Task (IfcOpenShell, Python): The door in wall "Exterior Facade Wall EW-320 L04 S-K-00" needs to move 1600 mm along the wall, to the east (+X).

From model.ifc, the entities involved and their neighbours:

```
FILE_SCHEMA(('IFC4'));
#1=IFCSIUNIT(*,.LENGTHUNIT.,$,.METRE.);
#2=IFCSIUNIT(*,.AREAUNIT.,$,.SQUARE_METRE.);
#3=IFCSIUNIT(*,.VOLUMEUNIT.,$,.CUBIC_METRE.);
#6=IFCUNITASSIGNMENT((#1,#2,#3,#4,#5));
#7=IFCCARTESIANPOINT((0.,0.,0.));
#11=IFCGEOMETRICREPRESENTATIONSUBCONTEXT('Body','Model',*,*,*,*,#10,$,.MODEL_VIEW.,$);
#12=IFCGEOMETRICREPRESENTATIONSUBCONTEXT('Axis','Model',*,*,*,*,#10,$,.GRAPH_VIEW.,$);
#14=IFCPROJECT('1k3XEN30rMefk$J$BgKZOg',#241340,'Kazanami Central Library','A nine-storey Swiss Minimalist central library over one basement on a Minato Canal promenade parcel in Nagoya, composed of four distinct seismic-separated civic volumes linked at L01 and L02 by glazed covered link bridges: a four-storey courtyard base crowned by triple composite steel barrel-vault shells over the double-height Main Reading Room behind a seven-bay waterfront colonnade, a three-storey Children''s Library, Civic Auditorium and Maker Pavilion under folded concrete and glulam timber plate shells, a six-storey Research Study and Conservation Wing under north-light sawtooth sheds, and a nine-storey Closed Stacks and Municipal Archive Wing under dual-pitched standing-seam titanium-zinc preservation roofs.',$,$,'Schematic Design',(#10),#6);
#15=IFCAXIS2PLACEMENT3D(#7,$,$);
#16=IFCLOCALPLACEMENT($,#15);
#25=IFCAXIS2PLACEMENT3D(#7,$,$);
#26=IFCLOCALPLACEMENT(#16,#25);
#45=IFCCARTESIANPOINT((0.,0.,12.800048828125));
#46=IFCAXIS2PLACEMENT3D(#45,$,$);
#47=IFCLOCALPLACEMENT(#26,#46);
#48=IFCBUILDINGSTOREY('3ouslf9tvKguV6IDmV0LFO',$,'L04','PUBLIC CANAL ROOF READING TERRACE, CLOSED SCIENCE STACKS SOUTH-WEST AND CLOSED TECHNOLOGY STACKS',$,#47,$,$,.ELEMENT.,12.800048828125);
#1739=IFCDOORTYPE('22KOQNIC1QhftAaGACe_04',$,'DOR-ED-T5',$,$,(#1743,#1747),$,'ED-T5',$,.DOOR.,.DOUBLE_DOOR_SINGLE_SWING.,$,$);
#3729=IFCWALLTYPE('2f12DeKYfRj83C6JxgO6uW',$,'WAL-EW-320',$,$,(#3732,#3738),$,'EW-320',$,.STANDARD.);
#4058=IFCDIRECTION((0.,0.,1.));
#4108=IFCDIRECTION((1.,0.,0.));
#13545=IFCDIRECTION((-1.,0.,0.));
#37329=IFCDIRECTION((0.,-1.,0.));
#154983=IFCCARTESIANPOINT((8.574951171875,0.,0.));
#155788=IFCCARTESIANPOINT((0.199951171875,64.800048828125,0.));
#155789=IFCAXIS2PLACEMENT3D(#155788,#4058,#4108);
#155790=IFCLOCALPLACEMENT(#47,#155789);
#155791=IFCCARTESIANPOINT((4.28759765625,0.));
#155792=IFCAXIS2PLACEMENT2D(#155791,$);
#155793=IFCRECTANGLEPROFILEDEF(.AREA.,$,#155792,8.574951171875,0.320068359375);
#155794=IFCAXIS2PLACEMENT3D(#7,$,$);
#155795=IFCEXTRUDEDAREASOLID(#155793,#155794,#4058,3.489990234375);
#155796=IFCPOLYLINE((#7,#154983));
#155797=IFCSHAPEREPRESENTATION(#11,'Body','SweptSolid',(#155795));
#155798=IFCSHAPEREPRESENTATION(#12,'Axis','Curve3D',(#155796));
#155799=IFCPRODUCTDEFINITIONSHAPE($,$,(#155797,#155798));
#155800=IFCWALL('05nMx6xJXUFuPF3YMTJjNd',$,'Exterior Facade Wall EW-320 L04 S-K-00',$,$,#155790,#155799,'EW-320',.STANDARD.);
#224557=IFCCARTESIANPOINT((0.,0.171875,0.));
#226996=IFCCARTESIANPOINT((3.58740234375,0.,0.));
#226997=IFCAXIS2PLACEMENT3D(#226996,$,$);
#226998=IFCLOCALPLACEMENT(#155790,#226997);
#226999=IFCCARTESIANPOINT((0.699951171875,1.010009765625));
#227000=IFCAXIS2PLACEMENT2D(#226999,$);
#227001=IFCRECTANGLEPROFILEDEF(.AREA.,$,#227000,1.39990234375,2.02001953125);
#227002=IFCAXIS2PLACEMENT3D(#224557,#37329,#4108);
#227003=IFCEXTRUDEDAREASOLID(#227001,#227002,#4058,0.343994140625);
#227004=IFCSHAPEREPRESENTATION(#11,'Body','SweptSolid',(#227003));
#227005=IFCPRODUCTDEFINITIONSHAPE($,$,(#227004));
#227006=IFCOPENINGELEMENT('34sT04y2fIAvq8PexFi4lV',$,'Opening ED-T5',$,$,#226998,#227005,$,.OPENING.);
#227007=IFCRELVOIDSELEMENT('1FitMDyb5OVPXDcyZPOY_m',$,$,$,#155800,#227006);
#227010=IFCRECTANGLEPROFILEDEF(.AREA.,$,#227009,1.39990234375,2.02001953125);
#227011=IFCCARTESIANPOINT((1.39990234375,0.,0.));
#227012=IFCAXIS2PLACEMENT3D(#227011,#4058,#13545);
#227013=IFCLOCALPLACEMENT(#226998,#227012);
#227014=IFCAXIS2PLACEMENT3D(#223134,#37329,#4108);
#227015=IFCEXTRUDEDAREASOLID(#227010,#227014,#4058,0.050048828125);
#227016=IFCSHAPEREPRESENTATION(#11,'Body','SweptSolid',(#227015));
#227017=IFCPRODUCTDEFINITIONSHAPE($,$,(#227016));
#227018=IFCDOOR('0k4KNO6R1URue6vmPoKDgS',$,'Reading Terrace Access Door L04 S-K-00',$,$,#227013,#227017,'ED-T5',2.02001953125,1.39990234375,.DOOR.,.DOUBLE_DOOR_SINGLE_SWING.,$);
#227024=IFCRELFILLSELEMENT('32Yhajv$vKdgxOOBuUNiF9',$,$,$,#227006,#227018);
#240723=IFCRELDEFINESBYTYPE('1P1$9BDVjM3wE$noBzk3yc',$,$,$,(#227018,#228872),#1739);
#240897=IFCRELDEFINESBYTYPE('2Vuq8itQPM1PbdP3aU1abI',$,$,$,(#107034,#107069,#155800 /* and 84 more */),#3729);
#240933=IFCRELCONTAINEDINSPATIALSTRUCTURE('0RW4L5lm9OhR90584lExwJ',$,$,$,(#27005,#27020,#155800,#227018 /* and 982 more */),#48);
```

```python
import ifcopenshell
import ifcopenshell.api.geometry
import ifcopenshell.util.placement
import ifcopenshell.util.unit

model = ifcopenshell.open("model.ifc")
unit_scale = ifcopenshell.util.unit.calculate_unit_scale(model)

door = model.by_id(227018)
opening = door.FillsVoids[0].RelatingOpeningElement
wall = opening.VoidsElements[0].RelatingBuildingElement

wall_matrix = ifcopenshell.util.placement.get_local_placement(wall.ObjectPlacement)
shift = wall_matrix[:3, 0] * 1.6 / unit_scale
before = ifcopenshell.util.placement.get_local_placement(door.ObjectPlacement)[:3, 3].copy()

# The door is placed relative to its opening, so it follows when the opening moves.
matrix = ifcopenshell.util.placement.get_local_placement(opening.ObjectPlacement)
matrix[:3, 3] += shift
ifcopenshell.api.geometry.edit_object_placement(
    model, product=opening, matrix=matrix, is_si=False, should_transform_children=True
)

after = ifcopenshell.util.placement.get_local_placement(door.ObjectPlacement)[:3, 3]
print("door moved by", (after - before).round(3) + 0.0)

model.write("model_updated.ifc")
```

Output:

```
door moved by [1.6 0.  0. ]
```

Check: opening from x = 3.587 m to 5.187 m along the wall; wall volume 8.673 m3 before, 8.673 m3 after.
